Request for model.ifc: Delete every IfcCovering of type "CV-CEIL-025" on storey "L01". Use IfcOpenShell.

First a look at what the model holds.

```python
import ifcopenshell
import ifcopenshell.util.element

model = ifcopenshell.open("model.ifc")
print(model.schema)
storey = next(s for s in model.by_type("IfcBuildingStorey") if s.Name == "L01")
coverings = [e for e in ifcopenshell.util.element.get_decomposition(storey) if e.is_a("IfcCovering")]
seen = {}
for e in coverings:
    element_type = ifcopenshell.util.element.get_type(e)
    name = element_type.Name if element_type not in (None, e) else None
    seen[name] = seen.get(name, 0) + 1
for name, count in sorted(seen.items(), key=str):
    print(count, "x", name)
```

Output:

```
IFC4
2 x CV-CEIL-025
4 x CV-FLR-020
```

```python
import ifcopenshell
import ifcopenshell.api.root
import ifcopenshell.util.element

model = ifcopenshell.open("model.ifc")

storey = next(s for s in model.by_type("IfcBuildingStorey") if s.Name == "L01")
coverings = [e for e in ifcopenshell.util.element.get_decomposition(storey) if e.is_a("IfcCovering")]
targets = [e for e in coverings if (t := ifcopenshell.util.element.get_type(e)) not in (None, e) and t.Name == "CV-CEIL-025"]

for e in targets:
    ifcopenshell.api.root.remove_product(model, product=e)
print(len(targets), "removed")

model.write("model_edited.ifc")
```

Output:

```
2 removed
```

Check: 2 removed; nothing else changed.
